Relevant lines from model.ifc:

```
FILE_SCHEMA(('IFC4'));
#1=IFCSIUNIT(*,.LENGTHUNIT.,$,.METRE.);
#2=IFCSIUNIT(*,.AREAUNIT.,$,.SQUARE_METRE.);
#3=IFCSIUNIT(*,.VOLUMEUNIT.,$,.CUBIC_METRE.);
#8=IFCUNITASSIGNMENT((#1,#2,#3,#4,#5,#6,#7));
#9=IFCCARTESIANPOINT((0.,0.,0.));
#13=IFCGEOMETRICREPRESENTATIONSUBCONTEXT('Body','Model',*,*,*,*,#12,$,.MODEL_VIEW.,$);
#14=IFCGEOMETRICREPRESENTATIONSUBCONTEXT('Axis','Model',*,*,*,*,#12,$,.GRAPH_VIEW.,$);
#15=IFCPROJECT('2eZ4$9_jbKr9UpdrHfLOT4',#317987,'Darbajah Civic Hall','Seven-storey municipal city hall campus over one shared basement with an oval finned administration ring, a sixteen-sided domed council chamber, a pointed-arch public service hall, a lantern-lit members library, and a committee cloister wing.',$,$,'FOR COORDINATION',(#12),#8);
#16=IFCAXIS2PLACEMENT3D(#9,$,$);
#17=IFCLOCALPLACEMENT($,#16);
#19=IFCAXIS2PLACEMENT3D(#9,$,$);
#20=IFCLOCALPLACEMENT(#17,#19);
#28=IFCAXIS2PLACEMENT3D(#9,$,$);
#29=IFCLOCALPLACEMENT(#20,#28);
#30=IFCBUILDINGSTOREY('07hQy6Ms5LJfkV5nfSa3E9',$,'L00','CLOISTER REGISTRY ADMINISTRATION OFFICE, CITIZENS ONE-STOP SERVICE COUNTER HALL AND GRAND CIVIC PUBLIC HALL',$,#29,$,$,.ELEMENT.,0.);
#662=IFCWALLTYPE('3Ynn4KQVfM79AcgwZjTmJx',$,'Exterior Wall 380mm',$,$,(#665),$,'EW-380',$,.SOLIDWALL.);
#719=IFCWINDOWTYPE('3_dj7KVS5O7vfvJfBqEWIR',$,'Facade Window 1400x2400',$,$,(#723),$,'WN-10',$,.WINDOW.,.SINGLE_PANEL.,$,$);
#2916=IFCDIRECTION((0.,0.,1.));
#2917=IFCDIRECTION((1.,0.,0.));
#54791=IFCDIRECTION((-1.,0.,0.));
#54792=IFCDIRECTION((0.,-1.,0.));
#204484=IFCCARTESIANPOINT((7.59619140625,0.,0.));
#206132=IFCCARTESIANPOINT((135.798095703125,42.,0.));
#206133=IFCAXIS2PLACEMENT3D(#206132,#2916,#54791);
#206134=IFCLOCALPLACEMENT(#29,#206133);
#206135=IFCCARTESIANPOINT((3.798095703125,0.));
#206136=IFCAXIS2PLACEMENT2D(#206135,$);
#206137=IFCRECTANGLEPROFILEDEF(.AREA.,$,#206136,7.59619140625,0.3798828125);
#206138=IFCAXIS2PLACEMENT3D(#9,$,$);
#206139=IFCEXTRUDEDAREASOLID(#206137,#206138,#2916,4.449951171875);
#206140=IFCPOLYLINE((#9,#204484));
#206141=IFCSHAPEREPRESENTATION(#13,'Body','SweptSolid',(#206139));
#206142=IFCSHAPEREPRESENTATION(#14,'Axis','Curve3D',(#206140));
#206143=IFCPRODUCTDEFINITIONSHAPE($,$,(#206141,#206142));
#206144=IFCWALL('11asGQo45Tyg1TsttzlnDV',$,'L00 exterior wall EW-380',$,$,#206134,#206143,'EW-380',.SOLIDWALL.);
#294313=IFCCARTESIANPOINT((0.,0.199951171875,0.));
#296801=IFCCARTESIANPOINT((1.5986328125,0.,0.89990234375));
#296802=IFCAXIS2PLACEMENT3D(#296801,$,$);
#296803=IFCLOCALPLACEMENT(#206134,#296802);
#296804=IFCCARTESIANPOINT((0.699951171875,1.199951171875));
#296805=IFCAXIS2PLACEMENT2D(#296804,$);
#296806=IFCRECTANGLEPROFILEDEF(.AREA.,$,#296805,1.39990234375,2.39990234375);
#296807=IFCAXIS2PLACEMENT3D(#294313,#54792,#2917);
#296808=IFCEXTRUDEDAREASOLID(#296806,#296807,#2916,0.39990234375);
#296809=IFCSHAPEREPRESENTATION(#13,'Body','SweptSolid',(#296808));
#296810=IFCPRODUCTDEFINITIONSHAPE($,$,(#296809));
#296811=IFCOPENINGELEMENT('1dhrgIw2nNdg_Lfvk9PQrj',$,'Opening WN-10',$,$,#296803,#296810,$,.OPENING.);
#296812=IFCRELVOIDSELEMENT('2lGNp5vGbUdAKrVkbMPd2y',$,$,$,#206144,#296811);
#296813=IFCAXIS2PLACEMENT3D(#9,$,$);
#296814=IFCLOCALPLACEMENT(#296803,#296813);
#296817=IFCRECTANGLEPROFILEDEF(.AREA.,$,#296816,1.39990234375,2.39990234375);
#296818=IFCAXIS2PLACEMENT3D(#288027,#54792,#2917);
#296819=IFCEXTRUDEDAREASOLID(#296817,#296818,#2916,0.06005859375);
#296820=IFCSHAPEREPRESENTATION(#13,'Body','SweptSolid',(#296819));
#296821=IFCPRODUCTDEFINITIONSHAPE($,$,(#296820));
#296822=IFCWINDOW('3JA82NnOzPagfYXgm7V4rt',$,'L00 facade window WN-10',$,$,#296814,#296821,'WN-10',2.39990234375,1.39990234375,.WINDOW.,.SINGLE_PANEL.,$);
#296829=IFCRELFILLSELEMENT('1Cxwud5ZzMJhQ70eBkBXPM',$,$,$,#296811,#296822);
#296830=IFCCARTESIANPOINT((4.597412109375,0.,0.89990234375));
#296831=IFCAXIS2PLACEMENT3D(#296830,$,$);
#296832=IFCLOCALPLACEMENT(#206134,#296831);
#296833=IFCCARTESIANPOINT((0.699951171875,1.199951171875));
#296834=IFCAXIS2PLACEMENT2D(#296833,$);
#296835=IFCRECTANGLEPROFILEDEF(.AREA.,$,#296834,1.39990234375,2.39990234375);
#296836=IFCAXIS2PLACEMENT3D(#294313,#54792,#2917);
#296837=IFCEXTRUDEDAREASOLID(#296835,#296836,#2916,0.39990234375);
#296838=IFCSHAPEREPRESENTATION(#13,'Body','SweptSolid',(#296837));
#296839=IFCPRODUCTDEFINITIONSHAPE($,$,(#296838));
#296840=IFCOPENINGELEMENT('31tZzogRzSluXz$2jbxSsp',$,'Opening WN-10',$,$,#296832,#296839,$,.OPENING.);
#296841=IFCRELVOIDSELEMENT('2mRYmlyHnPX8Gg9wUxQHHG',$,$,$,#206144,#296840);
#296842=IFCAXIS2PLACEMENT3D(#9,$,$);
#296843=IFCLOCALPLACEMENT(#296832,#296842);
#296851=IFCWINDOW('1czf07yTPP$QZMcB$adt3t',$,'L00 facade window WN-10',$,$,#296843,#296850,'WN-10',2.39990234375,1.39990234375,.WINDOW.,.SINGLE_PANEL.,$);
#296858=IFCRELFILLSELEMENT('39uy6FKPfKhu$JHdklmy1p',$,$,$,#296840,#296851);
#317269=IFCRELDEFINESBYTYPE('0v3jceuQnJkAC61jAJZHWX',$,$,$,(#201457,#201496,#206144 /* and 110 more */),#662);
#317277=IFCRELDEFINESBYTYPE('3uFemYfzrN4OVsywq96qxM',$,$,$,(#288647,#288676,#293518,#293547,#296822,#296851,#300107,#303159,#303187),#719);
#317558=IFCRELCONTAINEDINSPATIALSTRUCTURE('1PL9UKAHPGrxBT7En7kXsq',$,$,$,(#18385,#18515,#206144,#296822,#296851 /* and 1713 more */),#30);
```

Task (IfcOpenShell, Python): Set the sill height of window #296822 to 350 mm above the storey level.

```python
import numpy as np
import ifcopenshell
import ifcopenshell.api.geometry
import ifcopenshell.geom
import ifcopenshell.util.element
import ifcopenshell.util.placement
import ifcopenshell.util.shape
import ifcopenshell.util.unit

model = ifcopenshell.open("model.ifc")
unit_scale = ifcopenshell.util.unit.calculate_unit_scale(model)

window = model.by_id(296822)
opening = window.FillsVoids[0].RelatingOpeningElement
storey = ifcopenshell.util.element.get_container(window, ifc_class="IfcBuildingStorey")
level = ifcopenshell.util.placement.get_local_placement(storey.ObjectPlacement)[2, 3]

# The opening's origin need not be at the sill, so measure its lowest point.
shape = ifcopenshell.geom.create_shape(ifcopenshell.geom.settings(), opening)
bottom = ifcopenshell.util.shape.get_shape_bottom_elevation(shape, shape.geometry) / unit_scale
dz = level + 0.35 - bottom

shift = np.array([0.0, 0.0, dz])
# The window is placed relative to its opening, so it follows when the opening moves.
matrix = ifcopenshell.util.placement.get_local_placement(opening.ObjectPlacement)
matrix[:3, 3] += shift
ifcopenshell.api.geometry.edit_object_placement(
    model, product=opening, matrix=matrix, is_si=False, should_transform_children=True
)

print(f"moved by {dz * unit_scale:+.3f} m")

model.write("model_rev.ifc")
```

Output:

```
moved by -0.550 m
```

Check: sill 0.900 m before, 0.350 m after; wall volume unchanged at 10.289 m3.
